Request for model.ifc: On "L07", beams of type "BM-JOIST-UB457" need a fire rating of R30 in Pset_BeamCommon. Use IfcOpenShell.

First a look at what the model holds.

```python
import ifcopenshell
import ifcopenshell.util.element

model = ifcopenshell.open("model.ifc")
print(model.schema)
storey = next(s for s in model.by_type("IfcBuildingStorey") if s.Name == "L07")
beams = [e for e in ifcopenshell.util.element.get_decomposition(storey) if e.is_a("IfcBeam")]
seen = {}
for e in beams:
    element_type = ifcopenshell.util.element.get_type(e)
    key = (element_type.Name if element_type != e and element_type else None, ifcopenshell.util.element.get_pset(e, "Pset_BeamCommon", "FireRating"))
    seen[key] = seen.get(key, 0) + 1
for (name, value), count in sorted(seen.items(), key=str):
    print(count, "x", name, "|", value)
```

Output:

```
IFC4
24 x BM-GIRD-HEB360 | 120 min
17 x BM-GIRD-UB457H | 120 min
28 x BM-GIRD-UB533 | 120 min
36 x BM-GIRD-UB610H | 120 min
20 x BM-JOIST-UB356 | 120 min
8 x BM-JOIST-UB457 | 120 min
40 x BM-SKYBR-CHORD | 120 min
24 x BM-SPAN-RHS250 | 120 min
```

```python
import ifcopenshell
import ifcopenshell.api.pset
import ifcopenshell.util.element

model = ifcopenshell.open("model.ifc")

storey = next(s for s in model.by_type("IfcBuildingStorey") if s.Name == "L07")
beams = [e for e in ifcopenshell.util.element.get_decomposition(storey) if e.is_a("IfcBeam")]

count = 0
for e in beams:
    element_type = ifcopenshell.util.element.get_type(e)
    if element_type in (None, e) or element_type.Name != "BM-JOIST-UB457":
        continue
    # add_pset returns the element's existing set when there is one.
    pset = ifcopenshell.api.pset.add_pset(model, product=e, name="Pset_BeamCommon")
    ifcopenshell.api.pset.edit_pset(model, pset=pset, properties={"FireRating": "R30"})
    count += 1

print(count, "beams updated")

model.write("model_v2.ifc")
```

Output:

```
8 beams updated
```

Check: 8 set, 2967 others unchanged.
